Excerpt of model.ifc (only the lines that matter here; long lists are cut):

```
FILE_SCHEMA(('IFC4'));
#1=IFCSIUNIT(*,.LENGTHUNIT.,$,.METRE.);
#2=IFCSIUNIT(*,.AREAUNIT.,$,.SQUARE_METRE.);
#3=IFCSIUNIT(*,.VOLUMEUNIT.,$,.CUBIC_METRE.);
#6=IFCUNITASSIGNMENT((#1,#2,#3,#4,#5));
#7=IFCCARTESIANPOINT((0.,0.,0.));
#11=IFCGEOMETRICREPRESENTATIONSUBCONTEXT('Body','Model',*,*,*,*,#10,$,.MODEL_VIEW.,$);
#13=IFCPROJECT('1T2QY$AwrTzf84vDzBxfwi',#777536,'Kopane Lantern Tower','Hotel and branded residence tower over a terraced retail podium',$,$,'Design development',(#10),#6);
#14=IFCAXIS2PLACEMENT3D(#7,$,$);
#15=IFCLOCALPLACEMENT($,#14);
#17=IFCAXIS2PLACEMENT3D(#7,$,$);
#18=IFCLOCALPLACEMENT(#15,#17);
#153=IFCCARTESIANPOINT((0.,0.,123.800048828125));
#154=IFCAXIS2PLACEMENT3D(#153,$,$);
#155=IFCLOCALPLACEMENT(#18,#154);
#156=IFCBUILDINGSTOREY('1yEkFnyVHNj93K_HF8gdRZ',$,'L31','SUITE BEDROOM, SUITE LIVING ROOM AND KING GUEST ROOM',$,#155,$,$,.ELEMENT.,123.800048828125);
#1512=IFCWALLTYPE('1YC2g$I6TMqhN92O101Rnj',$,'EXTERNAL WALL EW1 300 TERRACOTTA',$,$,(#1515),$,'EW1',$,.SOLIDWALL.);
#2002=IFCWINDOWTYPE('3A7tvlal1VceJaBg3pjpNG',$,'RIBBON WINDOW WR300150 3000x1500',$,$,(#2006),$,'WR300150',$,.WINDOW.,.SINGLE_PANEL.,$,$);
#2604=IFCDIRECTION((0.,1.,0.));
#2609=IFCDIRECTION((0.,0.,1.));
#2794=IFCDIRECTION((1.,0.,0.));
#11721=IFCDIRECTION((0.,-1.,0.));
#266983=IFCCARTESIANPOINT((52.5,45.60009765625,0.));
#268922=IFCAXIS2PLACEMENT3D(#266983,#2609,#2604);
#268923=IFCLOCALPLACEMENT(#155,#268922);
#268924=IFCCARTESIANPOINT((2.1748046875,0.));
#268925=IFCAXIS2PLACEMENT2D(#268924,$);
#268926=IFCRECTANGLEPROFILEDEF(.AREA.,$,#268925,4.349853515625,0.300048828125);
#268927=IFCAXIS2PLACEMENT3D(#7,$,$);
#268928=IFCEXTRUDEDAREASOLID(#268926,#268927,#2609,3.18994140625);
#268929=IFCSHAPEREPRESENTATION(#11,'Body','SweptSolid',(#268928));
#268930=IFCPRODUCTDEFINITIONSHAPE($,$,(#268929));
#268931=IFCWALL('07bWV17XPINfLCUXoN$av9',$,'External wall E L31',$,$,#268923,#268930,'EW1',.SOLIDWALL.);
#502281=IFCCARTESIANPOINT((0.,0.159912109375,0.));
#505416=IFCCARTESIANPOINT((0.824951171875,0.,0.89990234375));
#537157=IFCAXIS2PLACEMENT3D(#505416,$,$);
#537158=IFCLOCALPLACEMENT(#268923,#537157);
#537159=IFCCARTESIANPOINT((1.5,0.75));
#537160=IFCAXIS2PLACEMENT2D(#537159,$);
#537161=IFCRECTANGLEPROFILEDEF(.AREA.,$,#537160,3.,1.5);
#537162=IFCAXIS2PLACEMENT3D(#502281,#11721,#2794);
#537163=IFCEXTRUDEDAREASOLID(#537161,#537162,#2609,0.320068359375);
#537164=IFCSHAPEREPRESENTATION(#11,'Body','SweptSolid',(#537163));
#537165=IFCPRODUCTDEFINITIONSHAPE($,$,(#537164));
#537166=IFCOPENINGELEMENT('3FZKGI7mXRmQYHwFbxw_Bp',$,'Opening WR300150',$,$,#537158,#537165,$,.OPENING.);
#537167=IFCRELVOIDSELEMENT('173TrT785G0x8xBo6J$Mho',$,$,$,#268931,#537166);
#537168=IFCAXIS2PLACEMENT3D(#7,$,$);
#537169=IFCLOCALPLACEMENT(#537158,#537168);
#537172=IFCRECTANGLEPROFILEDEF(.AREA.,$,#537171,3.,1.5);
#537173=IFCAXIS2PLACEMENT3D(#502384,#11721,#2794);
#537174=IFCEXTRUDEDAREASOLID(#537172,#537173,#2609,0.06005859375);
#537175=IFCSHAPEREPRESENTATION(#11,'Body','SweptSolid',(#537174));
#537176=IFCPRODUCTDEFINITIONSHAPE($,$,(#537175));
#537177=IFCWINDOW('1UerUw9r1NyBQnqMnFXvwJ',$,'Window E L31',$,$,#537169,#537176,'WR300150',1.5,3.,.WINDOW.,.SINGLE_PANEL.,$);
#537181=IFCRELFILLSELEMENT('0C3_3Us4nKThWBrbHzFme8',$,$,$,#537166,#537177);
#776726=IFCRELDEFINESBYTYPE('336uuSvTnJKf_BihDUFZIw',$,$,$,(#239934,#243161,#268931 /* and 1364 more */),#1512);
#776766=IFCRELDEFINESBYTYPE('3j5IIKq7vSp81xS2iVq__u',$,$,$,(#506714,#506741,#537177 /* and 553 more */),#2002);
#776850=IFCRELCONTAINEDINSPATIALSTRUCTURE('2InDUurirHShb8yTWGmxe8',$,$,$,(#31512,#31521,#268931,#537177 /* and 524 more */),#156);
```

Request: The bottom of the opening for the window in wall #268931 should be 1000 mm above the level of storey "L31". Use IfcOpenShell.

```python
import numpy as np
import ifcopenshell
import ifcopenshell.api.geometry
import ifcopenshell.geom
import ifcopenshell.util.element
import ifcopenshell.util.placement
import ifcopenshell.util.shape
import ifcopenshell.util.unit

model = ifcopenshell.open("model.ifc")
unit_scale = ifcopenshell.util.unit.calculate_unit_scale(model)

window = model.by_guid("1UerUw9r1NyBQnqMnFXvwJ")
opening = window.FillsVoids[0].RelatingOpeningElement
storey = ifcopenshell.util.element.get_container(window, ifc_class="IfcBuildingStorey")
level = ifcopenshell.util.placement.get_local_placement(storey.ObjectPlacement)[2, 3]

# The opening's origin need not be at the sill, so measure its lowest point.
shape = ifcopenshell.geom.create_shape(ifcopenshell.geom.settings(), opening)
bottom = ifcopenshell.util.shape.get_shape_bottom_elevation(shape, shape.geometry) / unit_scale
dz = level + 1 / unit_scale - bottom

shift = np.array([0.0, 0.0, dz])
# The window is placed relative to its opening, so it follows when the opening moves.
matrix = ifcopenshell.util.placement.get_local_placement(opening.ObjectPlacement)
matrix[:3, 3] += shift
ifcopenshell.api.geometry.edit_object_placement(
    model, product=opening, matrix=matrix, is_si=False, should_transform_children=True
)

print(f"moved by {dz * unit_scale:+.3f} m")

model.write("model_edited.ifc")
```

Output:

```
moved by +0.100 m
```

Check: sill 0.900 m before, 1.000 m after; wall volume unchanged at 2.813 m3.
